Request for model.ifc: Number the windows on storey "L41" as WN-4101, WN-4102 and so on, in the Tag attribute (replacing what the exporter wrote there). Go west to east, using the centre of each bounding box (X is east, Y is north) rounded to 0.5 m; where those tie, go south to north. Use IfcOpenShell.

First a look at what the model holds.

```python
import ifcopenshell
import ifcopenshell.util.element
import ifcopenshell.util.placement

model = ifcopenshell.open("model.ifc")
print(model.schema)
storey = next(s for s in model.by_type("IfcBuildingStorey") if s.Name == "L41")
windows = [e for e in ifcopenshell.util.element.get_decomposition(storey) if e.is_a("IfcWindow")]
for e in sorted(windows, key=lambda e: e.id()):
    origin = ifcopenshell.util.placement.get_local_placement(e.ObjectPlacement)[:3, 3]
    print(e.id(), e.Tag, e.Name, origin.round(2) + 0.0, sep=" | ")
```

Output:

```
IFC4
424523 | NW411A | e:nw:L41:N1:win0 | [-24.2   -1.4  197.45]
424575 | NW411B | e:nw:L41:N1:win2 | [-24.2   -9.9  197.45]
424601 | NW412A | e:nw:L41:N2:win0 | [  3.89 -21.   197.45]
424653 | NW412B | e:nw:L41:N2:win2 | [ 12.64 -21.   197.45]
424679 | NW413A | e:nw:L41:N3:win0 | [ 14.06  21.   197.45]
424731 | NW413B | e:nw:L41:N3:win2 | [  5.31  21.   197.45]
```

```python
import ifcopenshell
import ifcopenshell.geom
import ifcopenshell.util.element
import ifcopenshell.util.shape

model = ifcopenshell.open("model.ifc")
settings = ifcopenshell.geom.settings()
settings.set("use-world-coords", True)


def centre(element):
    shape = ifcopenshell.geom.create_shape(settings, element)
    return ifcopenshell.util.shape.get_bbox_centroid(shape.geometry)


storey = next(s for s in model.by_type("IfcBuildingStorey") if s.Name == "L41")
windows = [e for e in ifcopenshell.util.element.get_decomposition(storey) if e.is_a("IfcWindow")]

# Insertion points can sit at a corner or the storey origin, so sort by the geometry (in metres).
centres = {e: centre(e) for e in windows}
windows.sort(key=lambda e: (round(centres[e][0] / 0.5), centres[e][1]))

for i, e in enumerate(windows, start=1):
    number = f"WN-41{i:02d}"
    e.Tag = number
    print(e.id(), number)

model.write("model_v2.ifc")
```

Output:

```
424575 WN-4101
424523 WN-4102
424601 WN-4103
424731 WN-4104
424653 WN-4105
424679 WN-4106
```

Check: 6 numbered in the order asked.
